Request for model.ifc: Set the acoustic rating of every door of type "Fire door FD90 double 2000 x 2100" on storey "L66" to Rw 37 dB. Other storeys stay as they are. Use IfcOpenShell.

First a look at what the model holds.

```python
import ifcopenshell
import ifcopenshell.util.element

model = ifcopenshell.open("model.ifc")
print(model.schema)
storey = next(s for s in model.by_type("IfcBuildingStorey") if s.Name == "L66")
doors = [e for e in ifcopenshell.util.element.get_decomposition(storey) if e.is_a("IfcDoor")]
seen = {}
for e in doors:
    element_type = ifcopenshell.util.element.get_type(e)
    key = (element_type.Name if element_type != e and element_type else None, ifcopenshell.util.element.get_pset(e, "Pset_DoorCommon", "AcousticRating"))
    seen[key] = seen.get(key, 0) + 1
for (name, value), count in sorted(seen.items(), key=str):
    print(count, "x", name, "|", value)
```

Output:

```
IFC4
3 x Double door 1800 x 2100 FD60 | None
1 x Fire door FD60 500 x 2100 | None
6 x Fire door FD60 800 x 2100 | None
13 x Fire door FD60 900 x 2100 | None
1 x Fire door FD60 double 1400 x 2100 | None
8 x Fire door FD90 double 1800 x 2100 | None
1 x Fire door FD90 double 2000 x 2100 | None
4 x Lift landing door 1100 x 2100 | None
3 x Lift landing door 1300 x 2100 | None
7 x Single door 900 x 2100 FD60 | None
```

```python
import ifcopenshell
import ifcopenshell.api.pset
import ifcopenshell.util.element

model = ifcopenshell.open("model.ifc")

storey = next(s for s in model.by_type("IfcBuildingStorey") if s.Name == "L66")
doors = [e for e in ifcopenshell.util.element.get_decomposition(storey) if e.is_a("IfcDoor")]

count = 0
for e in doors:
    element_type = ifcopenshell.util.element.get_type(e)
    if element_type in (None, e) or element_type.Name != "Fire door FD90 double 2000 x 2100":
        continue
    found = ifcopenshell.util.element.get_pset(e, "Pset_DoorCommon", should_inherit=False)
    if found:
        pset = model.by_id(found["id"])
        if len(ifcopenshell.util.element.get_elements_by_pset(pset)) > 1:
            pset = ifcopenshell.api.pset.unshare_pset(model, products=[e], pset=pset)[0]
    else:
        pset = ifcopenshell.api.pset.add_pset(model, product=e, name="Pset_DoorCommon")
    ifcopenshell.api.pset.edit_pset(model, pset=pset, properties={"AcousticRating": "Rw 37 dB"})
    count += 1

print(count, "doors updated")

model.write("model_edited.ifc")
```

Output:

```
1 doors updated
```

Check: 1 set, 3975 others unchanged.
